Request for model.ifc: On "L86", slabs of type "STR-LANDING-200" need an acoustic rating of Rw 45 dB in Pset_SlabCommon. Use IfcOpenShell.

First a look at what the model holds.

```python
import ifcopenshell
import ifcopenshell.util.element

model = ifcopenshell.open("model.ifc")
print(model.schema)
storey = next(s for s in model.by_type("IfcBuildingStorey") if s.Name == "L86")
slabs = [e for e in ifcopenshell.util.element.get_decomposition(storey) if e.is_a("IfcSlab")]
seen = {}
for e in slabs:
    element_type = ifcopenshell.util.element.get_type(e)
    key = (element_type.Name if element_type != e and element_type else None, ifcopenshell.util.element.get_pset(e, "Pset_SlabCommon", "AcousticRating"))
    seen[key] = seen.get(key, 0) + 1
for (name, value), count in sorted(seen.items(), key=str):
    print(count, "x", name, "|", value)
```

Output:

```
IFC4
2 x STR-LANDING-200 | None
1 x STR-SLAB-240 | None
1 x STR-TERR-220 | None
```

```python
import ifcopenshell
import ifcopenshell.api.pset
import ifcopenshell.util.element

model = ifcopenshell.open("model.ifc")

storey = next(s for s in model.by_type("IfcBuildingStorey") if s.Name == "L86")
slabs = [e for e in ifcopenshell.util.element.get_decomposition(storey) if e.is_a("IfcSlab")]

count = 0
for e in slabs:
    element_type = ifcopenshell.util.element.get_type(e)
    if element_type in (None, e) or element_type.Name != "STR-LANDING-200":
        continue
    found = ifcopenshell.util.element.get_pset(e, "Pset_SlabCommon", should_inherit=False)
    if found:
        pset = model.by_id(found["id"])
        if len(ifcopenshell.util.element.get_elements_by_pset(pset)) > 1:
            pset = ifcopenshell.api.pset.unshare_pset(model, products=[e], pset=pset)[0]
    else:
        pset = ifcopenshell.api.pset.add_pset(model, product=e, name="Pset_SlabCommon")
    ifcopenshell.api.pset.edit_pset(model, pset=pset, properties={"AcousticRating": "Rw 45 dB"})
    count += 1

print(count, "slabs updated")

model.write("model_edited.ifc")
```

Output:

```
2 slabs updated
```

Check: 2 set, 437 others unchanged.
